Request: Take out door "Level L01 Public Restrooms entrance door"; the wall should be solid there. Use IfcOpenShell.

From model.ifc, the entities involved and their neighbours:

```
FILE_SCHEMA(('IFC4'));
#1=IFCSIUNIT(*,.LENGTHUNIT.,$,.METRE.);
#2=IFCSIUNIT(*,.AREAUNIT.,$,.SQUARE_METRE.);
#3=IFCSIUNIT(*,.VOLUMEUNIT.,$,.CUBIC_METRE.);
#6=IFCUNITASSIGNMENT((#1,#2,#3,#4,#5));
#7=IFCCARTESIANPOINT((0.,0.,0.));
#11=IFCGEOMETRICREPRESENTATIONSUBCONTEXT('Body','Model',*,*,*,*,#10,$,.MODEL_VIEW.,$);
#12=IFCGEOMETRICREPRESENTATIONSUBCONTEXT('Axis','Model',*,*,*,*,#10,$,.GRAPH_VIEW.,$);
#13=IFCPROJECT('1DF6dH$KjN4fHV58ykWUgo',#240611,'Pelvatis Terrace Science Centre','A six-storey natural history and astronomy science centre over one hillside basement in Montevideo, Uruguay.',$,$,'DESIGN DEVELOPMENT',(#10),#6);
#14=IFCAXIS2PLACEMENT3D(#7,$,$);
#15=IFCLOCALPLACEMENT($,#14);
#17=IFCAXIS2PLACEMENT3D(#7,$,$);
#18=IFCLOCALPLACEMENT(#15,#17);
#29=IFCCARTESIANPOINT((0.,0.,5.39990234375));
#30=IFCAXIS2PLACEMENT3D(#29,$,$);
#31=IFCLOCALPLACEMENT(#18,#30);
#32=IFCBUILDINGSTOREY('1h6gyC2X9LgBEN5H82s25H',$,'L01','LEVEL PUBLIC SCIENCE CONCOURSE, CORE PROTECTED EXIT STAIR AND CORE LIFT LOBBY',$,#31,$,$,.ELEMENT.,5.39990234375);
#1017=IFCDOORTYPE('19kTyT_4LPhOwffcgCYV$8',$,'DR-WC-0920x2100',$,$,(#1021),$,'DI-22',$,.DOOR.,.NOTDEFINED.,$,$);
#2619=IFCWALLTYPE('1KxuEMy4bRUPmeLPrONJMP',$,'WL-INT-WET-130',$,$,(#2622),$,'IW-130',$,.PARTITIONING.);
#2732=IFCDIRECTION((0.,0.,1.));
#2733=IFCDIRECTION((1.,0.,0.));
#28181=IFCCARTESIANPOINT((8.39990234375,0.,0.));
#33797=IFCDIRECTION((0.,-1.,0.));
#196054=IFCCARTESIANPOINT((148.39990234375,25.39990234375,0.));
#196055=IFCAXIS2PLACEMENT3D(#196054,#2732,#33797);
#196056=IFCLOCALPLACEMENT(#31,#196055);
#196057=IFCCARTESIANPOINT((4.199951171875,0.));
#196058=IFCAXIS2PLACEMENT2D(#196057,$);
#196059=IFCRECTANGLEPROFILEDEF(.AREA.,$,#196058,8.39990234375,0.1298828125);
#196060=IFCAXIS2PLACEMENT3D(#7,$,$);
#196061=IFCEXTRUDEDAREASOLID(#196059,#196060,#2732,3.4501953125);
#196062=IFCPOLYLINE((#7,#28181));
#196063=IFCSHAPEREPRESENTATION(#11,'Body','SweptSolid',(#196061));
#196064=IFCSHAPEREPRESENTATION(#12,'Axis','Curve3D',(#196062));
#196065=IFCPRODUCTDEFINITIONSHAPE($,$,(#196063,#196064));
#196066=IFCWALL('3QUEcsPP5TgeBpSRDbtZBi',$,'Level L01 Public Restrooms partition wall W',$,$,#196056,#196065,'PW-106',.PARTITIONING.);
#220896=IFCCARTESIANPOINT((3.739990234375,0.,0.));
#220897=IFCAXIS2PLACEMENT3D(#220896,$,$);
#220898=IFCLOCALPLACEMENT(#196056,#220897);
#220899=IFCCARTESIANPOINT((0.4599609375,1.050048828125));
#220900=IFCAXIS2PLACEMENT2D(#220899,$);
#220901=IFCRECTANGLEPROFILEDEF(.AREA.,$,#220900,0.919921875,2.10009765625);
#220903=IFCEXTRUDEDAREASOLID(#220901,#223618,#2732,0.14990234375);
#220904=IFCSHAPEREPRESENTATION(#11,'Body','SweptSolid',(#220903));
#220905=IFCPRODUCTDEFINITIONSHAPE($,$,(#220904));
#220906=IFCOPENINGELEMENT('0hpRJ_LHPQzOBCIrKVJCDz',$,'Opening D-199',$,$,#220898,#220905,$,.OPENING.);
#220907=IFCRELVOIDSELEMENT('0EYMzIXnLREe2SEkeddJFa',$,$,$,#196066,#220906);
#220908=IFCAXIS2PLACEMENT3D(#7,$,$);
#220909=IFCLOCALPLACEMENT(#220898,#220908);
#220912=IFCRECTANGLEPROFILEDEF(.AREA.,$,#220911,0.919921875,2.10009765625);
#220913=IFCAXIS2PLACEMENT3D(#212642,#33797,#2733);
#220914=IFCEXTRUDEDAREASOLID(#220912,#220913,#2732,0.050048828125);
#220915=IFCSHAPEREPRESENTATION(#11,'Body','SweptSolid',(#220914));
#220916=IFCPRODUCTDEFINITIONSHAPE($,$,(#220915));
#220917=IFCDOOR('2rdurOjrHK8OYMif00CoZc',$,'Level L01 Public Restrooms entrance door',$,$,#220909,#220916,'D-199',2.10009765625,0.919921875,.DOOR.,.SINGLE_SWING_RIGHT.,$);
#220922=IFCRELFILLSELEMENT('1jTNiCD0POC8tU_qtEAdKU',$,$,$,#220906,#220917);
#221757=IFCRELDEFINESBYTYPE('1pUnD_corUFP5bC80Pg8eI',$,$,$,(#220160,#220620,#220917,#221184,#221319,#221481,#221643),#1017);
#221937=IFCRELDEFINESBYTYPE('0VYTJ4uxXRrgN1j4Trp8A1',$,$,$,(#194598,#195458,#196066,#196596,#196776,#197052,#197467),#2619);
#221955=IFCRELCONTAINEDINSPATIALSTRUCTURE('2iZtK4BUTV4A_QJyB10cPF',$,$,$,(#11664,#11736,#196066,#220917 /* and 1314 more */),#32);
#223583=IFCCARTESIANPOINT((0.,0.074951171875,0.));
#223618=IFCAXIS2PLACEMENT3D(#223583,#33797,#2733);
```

```python
import ifcopenshell
import ifcopenshell.api.feature
import ifcopenshell.api.root
import ifcopenshell.geom
import ifcopenshell.util.shape

model = ifcopenshell.open("model.ifc")
settings = ifcopenshell.geom.settings()


def volume(element):
    """Net volume in cubic metres, openings subtracted."""
    shape = ifcopenshell.geom.create_shape(settings, element)
    return ifcopenshell.util.shape.get_volume(shape.geometry)


door = model.by_id(220917)
opening = door.FillsVoids[0].RelatingOpeningElement
wall = opening.VoidsElements[0].RelatingBuildingElement
before = volume(wall)

ifcopenshell.api.root.remove_product(model, product=door)
ifcopenshell.api.feature.remove_feature(model, feature=opening)

after = volume(wall)

print(f"wall volume {before:.3f} -> {after:.3f} m3")

model.write("model_v2.ifc")
```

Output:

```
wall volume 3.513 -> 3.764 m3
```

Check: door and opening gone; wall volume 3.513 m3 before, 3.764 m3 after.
